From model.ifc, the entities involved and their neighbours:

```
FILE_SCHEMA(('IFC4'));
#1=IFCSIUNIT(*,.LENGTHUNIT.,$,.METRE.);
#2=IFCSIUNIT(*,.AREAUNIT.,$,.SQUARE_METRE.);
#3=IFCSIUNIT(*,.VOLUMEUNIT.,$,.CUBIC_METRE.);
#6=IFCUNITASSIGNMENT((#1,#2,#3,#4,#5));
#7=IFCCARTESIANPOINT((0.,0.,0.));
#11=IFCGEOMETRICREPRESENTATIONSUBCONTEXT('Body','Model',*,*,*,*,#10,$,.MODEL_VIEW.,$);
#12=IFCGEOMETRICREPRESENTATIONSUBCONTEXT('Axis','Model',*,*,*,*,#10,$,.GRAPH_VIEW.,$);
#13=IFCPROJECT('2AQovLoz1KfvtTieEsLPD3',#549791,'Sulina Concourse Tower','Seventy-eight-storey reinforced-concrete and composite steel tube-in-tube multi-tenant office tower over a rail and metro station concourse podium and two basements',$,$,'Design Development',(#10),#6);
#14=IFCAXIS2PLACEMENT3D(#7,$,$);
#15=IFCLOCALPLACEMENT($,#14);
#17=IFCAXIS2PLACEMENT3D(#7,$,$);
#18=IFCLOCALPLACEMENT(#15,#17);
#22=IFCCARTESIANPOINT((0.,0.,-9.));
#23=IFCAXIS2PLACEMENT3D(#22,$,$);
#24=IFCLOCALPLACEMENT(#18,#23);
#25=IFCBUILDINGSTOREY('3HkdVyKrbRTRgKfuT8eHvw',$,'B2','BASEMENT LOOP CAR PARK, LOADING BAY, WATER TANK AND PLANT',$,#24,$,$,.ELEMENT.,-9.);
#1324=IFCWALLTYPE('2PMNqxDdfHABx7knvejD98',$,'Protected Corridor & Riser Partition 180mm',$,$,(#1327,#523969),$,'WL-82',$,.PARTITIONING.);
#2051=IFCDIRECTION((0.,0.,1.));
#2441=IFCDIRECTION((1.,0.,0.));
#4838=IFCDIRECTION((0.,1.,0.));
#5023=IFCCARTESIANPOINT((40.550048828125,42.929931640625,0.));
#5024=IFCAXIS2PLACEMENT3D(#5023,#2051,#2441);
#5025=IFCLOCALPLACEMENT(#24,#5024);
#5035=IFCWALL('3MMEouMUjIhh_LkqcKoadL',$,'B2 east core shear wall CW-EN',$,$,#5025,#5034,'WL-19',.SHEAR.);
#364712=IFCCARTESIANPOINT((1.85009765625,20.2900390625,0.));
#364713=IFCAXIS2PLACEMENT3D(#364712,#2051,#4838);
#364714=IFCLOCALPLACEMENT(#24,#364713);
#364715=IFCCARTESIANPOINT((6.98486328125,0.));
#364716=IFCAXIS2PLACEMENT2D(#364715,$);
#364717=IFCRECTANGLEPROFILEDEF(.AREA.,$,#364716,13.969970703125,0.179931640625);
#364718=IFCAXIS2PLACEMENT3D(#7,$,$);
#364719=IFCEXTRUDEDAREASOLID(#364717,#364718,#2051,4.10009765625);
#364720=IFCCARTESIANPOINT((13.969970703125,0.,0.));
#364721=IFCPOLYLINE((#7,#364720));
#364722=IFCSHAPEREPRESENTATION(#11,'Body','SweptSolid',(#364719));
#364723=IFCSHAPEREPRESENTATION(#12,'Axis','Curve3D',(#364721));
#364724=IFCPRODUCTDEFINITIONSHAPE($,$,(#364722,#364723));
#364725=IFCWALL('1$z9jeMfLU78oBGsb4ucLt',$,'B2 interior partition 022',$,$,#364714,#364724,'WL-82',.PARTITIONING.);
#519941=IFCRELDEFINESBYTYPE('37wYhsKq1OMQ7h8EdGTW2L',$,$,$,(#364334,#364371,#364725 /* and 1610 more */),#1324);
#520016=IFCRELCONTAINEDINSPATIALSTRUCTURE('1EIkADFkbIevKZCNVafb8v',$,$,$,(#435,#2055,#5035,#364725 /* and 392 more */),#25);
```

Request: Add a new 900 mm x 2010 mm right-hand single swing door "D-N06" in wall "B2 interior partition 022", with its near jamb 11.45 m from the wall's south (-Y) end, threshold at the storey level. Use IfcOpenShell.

```python
import numpy as np
import ifcopenshell
import ifcopenshell.api.feature
import ifcopenshell.api.geometry
import ifcopenshell.api.root
import ifcopenshell.api.spatial
import ifcopenshell.geom
import ifcopenshell.util.element
import ifcopenshell.util.placement
import ifcopenshell.util.representation
import ifcopenshell.util.shape
import ifcopenshell.util.unit

model = ifcopenshell.open("model.ifc")
unit_scale = ifcopenshell.util.unit.calculate_unit_scale(model)
settings = ifcopenshell.geom.settings()


def volume(element):
    """Net volume in cubic metres, openings subtracted."""
    shape = ifcopenshell.geom.create_shape(settings, element)
    return ifcopenshell.util.shape.get_volume(shape.geometry)


wall = model.by_guid("1$z9jeMfLU78oBGsb4ucLt")
storey = ifcopenshell.util.element.get_container(wall, ifc_class="IfcBuildingStorey")
context = ifcopenshell.util.representation.get_context(model, "Model", "Body", "MODEL_VIEW")
before = volume(wall)

width, height, from_end, sill = 0.9, 2.01, 11.45, 0.0  # metres

# The wall runs along its own X axis, and the end named is its -X end.
wall_shape = ifcopenshell.geom.create_shape(settings, wall)
x, y, z = ifcopenshell.util.shape.get_vertices(wall_shape.geometry).T
start = x.min() + from_end
face, thickness = float(y.min()), float(y.max() - y.min())
wall_matrix = ifcopenshell.util.placement.get_local_placement(wall.ObjectPlacement)
level = ifcopenshell.util.placement.get_local_placement(storey.ObjectPlacement)[2, 3]


def in_wall(x, y):
    """Placement at x, y metres in the wall's axes, at sill height."""
    matrix = wall_matrix.copy()
    matrix[:, 3] = wall_matrix @ np.array([x / unit_scale, y / unit_scale, 0.0, 1.0])
    matrix[2, 3] = level + sill / unit_scale
    return matrix


# Opening: a box that overshoots both wall faces by 50 mm.
opening = ifcopenshell.api.root.create_entity(model, ifc_class="IfcOpeningElement", predefined_type="OPENING")
box = ifcopenshell.api.geometry.add_wall_representation(
    model, context=context, length=width, height=height, thickness=thickness + 0.1
)
ifcopenshell.api.geometry.assign_representation(model, product=opening, representation=box)
ifcopenshell.api.geometry.edit_object_placement(model, product=opening, matrix=in_wall(start, face - 0.05), is_si=False)
ifcopenshell.api.feature.add_feature(model, feature=opening, element=wall)

door = ifcopenshell.api.root.create_entity(model, ifc_class="IfcDoor", name="D-N06", predefined_type="DOOR")
door.OverallWidth, door.OverallHeight = width / unit_scale, height / unit_scale
door.OperationType = "SINGLE_SWING_RIGHT"
body = ifcopenshell.api.geometry.add_door_representation(
    model,
    context=context,
    overall_width=door.OverallWidth,
    overall_height=door.OverallHeight,
    operation_type="SINGLE_SWING_RIGHT",
    lining_properties={"LiningDepth": thickness / unit_scale, "ThresholdDepth": thickness / unit_scale},
)
ifcopenshell.api.geometry.assign_representation(model, product=door, representation=body)
ifcopenshell.api.spatial.assign_container(model, products=[door], relating_structure=storey)
ifcopenshell.api.feature.add_filling(model, opening=opening, element=door)

# The lining spans the wall, so the door starts at the wall face.
ifcopenshell.api.geometry.edit_object_placement(model, product=door, matrix=in_wall(start, face), is_si=False)

after = volume(wall)

print(f"wall volume {before:.3f} -> {after:.3f} m3")

model.write("model_updated.ifc")
```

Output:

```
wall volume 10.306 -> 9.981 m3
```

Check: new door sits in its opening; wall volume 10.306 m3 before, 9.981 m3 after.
